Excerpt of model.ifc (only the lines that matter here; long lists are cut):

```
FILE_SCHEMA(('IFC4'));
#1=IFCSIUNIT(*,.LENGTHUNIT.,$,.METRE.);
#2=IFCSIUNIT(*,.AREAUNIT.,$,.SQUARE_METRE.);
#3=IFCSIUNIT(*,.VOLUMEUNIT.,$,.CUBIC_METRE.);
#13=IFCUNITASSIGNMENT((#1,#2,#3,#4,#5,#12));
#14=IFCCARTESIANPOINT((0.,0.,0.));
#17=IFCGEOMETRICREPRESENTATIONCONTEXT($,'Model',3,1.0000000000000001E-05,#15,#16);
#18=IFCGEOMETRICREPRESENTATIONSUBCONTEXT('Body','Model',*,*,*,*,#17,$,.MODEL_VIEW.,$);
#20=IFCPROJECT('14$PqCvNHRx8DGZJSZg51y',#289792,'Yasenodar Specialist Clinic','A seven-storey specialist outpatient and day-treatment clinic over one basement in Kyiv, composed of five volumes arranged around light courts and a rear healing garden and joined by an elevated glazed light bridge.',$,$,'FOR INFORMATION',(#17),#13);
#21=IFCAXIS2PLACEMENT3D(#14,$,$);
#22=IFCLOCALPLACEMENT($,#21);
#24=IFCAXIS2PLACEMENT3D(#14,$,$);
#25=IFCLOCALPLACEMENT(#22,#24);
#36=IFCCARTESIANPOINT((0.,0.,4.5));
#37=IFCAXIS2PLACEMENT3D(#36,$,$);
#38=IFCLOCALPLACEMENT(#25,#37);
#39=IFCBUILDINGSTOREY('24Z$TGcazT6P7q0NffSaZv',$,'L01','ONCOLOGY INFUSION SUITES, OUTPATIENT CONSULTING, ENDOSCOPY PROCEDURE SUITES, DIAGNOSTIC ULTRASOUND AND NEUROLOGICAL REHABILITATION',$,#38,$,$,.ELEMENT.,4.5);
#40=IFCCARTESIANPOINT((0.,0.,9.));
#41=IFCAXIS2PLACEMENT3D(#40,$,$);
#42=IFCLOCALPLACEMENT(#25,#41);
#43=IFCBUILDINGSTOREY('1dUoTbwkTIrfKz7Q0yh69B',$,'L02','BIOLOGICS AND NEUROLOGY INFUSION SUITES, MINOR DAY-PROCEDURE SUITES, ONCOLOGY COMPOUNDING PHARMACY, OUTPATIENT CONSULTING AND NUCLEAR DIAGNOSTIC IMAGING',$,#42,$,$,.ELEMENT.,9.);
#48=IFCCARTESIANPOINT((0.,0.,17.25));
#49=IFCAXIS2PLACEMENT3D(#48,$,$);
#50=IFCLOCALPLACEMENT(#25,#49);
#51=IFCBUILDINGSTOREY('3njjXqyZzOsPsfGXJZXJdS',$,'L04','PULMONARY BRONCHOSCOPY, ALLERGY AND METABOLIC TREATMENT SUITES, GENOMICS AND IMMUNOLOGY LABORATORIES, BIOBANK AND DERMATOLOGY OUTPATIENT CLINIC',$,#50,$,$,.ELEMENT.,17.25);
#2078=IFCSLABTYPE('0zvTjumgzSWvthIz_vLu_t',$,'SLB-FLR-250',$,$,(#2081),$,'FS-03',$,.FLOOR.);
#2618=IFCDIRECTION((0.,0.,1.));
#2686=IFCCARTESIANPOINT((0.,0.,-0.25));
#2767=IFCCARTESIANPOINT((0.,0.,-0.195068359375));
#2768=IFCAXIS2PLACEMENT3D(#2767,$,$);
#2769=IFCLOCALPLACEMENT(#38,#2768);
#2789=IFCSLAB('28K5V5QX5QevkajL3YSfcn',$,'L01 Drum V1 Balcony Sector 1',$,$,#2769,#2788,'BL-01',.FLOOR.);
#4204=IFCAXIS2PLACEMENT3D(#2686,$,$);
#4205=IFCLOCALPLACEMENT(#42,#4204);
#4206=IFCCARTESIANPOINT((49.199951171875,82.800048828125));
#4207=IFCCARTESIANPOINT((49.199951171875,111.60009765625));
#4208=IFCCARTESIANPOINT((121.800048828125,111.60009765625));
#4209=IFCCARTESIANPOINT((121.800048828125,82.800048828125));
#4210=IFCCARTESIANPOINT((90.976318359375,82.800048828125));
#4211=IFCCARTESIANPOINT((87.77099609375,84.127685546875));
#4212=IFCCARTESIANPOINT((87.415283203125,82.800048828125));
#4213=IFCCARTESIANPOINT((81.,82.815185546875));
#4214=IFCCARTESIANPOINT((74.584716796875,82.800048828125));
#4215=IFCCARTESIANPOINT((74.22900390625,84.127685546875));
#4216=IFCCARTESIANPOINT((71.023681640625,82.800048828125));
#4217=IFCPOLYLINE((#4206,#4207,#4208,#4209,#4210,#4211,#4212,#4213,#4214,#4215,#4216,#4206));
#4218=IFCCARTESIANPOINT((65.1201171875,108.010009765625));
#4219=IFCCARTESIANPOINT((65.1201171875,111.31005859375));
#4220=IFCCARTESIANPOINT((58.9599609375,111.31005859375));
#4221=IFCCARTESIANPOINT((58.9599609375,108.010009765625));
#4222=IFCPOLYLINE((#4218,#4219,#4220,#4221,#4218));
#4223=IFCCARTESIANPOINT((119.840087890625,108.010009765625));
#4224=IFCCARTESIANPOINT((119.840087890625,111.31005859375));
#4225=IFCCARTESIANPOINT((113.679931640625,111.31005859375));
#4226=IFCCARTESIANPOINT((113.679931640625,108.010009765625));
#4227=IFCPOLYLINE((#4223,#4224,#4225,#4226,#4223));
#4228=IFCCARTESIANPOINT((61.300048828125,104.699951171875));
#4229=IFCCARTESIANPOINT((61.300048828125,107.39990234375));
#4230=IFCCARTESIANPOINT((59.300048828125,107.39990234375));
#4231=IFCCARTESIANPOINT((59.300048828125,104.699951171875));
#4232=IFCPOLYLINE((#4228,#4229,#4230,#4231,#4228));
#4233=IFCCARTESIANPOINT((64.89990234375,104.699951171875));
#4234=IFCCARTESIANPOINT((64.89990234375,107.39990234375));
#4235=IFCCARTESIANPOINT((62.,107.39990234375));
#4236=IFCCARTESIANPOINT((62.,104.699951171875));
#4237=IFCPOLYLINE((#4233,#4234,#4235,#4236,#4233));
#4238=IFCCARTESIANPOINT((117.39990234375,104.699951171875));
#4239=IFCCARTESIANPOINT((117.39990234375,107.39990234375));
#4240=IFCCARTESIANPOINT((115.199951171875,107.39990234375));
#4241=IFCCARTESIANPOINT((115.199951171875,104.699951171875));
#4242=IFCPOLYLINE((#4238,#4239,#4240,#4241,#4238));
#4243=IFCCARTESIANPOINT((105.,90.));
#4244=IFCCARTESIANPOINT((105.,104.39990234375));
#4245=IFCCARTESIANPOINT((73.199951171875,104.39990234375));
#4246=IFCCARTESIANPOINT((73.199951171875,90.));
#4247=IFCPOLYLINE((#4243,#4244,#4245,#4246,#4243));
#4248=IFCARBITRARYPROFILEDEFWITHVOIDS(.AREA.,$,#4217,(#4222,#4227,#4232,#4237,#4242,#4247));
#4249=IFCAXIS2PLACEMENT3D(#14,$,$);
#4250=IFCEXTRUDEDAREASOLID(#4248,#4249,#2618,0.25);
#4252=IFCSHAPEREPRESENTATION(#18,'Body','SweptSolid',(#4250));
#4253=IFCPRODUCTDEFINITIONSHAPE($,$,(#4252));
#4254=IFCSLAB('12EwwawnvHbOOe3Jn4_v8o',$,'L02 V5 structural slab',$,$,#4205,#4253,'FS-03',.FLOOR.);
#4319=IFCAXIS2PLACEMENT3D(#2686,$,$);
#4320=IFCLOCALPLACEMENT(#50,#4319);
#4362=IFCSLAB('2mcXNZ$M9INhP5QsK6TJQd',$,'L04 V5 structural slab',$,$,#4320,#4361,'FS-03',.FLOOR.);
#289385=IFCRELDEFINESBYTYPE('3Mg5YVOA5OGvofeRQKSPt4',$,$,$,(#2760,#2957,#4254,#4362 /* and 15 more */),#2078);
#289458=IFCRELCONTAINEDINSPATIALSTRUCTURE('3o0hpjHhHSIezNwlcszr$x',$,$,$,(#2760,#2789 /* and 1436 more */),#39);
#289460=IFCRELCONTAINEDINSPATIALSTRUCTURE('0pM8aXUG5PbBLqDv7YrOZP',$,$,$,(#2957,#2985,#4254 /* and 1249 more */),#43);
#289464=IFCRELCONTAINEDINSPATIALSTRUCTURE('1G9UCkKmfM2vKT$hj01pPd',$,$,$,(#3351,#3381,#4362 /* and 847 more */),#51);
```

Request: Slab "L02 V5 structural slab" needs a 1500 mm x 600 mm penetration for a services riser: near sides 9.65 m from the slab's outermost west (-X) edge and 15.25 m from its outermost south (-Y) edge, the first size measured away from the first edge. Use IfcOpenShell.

```python
import numpy as np
import ifcopenshell
import ifcopenshell.api.feature
import ifcopenshell.api.geometry
import ifcopenshell.api.root
import ifcopenshell.geom
import ifcopenshell.util.placement
import ifcopenshell.util.representation
import ifcopenshell.util.shape
import ifcopenshell.util.unit

model = ifcopenshell.open("model.ifc")
unit_scale = ifcopenshell.util.unit.calculate_unit_scale(model)
settings = ifcopenshell.geom.settings()


def volume(element):
    """Net volume in cubic metres, openings subtracted."""
    shape = ifcopenshell.geom.create_shape(settings, element)
    return ifcopenshell.util.shape.get_volume(shape.geometry)


slab = model.by_guid("12EwwawnvHbOOe3Jn4_v8o")
before = volume(slab)

# Extent in the slab's own axes, in metres. The edges named are its -X and -Y sides.
slab_shape = ifcopenshell.geom.create_shape(settings, slab)
vertices = ifcopenshell.util.shape.get_vertices(slab_shape.geometry)
x_min, y_min, bottom = vertices.min(axis=0)
top = vertices[:, 2].max()

opening = ifcopenshell.api.root.create_entity(model, ifc_class="IfcOpeningElement", name="Services riser opening", predefined_type="OPENING")
context = ifcopenshell.util.representation.get_context(model, "Model", "Body", "MODEL_VIEW")
width, depth = 1.5, 0.6
outline = [(0.0, 0.0), (width, 0.0), (width, depth), (0.0, depth), (0.0, 0.0)]
# Overshoot both faces by 50 mm so the cut is clean.
shape = ifcopenshell.api.geometry.add_slab_representation(
    model, context=context, depth=top - bottom + 0.1, polyline=outline
)
ifcopenshell.api.geometry.assign_representation(model, product=opening, representation=shape)

matrix = ifcopenshell.util.placement.get_local_placement(slab.ObjectPlacement)
matrix[:, 3] = matrix @ np.append(np.array([x_min + 9.65, y_min + 15.25, bottom - 0.05]) / unit_scale, 1.0)
ifcopenshell.api.geometry.edit_object_placement(model, product=opening, matrix=matrix, is_si=False)
ifcopenshell.api.feature.add_feature(model, feature=opening, element=slab)

after = volume(slab)

print(f"slab volume {before:.3f} -> {after:.3f} m3")

model.write("model_rev.ifc")
```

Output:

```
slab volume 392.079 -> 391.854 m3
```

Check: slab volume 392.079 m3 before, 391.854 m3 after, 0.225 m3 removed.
